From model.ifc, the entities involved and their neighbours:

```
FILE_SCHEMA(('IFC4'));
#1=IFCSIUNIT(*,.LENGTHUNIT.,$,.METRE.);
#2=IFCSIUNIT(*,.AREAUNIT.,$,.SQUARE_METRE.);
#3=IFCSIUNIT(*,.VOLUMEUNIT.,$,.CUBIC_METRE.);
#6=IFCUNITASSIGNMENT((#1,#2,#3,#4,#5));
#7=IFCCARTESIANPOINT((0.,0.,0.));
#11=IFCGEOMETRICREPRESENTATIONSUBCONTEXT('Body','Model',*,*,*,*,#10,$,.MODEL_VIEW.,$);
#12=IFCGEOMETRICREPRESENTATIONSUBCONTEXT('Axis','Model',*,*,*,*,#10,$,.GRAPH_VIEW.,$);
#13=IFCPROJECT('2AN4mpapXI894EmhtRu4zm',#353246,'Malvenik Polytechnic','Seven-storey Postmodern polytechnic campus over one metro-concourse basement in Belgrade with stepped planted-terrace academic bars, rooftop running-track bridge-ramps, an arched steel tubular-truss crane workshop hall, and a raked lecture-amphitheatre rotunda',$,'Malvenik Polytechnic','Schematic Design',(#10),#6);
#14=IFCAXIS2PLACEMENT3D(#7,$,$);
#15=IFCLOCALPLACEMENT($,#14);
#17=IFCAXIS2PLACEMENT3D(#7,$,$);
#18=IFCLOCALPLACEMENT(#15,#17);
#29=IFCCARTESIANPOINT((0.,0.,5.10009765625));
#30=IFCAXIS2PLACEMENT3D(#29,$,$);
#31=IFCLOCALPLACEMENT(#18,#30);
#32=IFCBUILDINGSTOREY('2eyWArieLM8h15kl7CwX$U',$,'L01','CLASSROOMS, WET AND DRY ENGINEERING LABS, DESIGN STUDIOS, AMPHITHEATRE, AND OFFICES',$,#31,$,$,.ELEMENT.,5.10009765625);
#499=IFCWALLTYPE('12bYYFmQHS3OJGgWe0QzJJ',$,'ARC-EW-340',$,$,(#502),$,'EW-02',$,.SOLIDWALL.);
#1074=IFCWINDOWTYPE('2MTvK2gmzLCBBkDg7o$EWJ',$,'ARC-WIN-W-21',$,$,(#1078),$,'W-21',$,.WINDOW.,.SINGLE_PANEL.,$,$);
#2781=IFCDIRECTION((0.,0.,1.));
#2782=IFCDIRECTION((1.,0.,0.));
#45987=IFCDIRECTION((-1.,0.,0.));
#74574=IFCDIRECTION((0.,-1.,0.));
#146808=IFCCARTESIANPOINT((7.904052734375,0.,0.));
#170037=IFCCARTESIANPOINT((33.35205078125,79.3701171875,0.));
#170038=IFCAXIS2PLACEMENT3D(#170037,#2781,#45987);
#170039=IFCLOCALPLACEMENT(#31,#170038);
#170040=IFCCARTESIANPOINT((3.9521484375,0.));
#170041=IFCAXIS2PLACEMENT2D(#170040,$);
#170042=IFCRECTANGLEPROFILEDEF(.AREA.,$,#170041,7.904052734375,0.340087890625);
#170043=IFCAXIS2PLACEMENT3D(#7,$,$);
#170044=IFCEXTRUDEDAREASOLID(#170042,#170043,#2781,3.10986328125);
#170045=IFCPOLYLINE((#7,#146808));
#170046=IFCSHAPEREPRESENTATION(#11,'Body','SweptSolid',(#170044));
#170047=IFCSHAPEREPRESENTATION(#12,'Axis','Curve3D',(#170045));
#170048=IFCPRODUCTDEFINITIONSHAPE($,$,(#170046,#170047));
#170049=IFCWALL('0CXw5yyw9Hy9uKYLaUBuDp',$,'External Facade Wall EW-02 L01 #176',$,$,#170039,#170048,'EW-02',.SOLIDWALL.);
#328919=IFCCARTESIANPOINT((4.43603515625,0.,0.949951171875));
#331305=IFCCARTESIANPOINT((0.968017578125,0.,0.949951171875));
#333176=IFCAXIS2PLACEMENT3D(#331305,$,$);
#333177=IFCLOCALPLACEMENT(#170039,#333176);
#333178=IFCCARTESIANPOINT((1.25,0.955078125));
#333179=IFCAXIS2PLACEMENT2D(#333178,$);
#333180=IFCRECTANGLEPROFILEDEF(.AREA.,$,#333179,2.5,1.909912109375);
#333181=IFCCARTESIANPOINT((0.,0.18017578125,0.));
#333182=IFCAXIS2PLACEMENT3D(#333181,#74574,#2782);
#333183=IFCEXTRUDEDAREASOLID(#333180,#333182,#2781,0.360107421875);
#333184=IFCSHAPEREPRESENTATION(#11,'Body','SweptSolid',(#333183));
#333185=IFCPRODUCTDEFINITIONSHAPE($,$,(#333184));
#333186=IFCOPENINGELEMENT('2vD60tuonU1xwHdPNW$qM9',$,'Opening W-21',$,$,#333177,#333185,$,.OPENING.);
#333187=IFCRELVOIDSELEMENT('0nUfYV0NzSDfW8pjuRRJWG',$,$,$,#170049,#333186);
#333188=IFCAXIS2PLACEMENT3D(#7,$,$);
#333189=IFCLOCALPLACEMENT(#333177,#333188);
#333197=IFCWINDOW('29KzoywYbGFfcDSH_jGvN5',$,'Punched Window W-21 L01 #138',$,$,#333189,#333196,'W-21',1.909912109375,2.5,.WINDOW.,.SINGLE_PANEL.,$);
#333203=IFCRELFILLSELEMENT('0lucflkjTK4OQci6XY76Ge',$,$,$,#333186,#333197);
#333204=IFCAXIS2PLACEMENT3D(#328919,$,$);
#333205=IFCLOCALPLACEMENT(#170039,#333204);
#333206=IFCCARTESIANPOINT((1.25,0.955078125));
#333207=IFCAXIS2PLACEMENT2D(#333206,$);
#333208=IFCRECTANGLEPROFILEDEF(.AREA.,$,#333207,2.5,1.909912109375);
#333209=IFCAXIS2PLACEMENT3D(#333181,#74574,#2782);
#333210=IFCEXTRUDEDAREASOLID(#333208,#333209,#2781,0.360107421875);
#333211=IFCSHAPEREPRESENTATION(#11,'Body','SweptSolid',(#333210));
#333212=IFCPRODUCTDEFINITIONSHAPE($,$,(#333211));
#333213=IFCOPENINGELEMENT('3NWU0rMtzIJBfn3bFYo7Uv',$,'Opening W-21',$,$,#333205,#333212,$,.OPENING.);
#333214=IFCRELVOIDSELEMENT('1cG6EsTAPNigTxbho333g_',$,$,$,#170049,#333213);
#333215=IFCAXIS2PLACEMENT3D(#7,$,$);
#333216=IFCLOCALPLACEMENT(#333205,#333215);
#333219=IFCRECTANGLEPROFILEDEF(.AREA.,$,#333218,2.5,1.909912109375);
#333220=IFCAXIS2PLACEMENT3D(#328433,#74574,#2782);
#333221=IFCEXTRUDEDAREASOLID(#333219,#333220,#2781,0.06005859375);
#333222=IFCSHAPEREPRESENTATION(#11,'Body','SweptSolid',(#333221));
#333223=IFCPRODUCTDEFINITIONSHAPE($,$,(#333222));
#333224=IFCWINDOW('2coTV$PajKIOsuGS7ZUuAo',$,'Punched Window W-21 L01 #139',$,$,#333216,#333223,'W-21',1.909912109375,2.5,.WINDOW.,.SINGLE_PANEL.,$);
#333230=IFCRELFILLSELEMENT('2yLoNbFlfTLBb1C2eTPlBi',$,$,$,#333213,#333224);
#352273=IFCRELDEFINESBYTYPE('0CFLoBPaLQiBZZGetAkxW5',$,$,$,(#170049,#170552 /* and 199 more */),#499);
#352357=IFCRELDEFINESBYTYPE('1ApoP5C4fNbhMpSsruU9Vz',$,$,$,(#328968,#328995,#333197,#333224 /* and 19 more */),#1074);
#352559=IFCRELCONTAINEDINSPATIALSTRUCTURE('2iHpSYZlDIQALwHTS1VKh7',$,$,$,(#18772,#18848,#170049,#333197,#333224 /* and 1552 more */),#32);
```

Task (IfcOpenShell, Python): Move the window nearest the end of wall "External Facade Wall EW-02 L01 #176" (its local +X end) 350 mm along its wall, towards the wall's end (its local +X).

```python
import ifcopenshell
import ifcopenshell.api.geometry
import ifcopenshell.util.placement

model = ifcopenshell.open("model.ifc")

window = model.by_guid("2coTV$PajKIOsuGS7ZUuAo")
opening = window.FillsVoids[0].RelatingOpeningElement
wall = opening.VoidsElements[0].RelatingBuildingElement

wall_matrix = ifcopenshell.util.placement.get_local_placement(wall.ObjectPlacement)
shift = wall_matrix[:3, 0] * 0.35
before = ifcopenshell.util.placement.get_local_placement(window.ObjectPlacement)[:3, 3].copy()

# The window is placed relative to its opening, so it follows when the opening moves.
matrix = ifcopenshell.util.placement.get_local_placement(opening.ObjectPlacement)
matrix[:3, 3] += shift
ifcopenshell.api.geometry.edit_object_placement(
    model, product=opening, matrix=matrix, is_si=False, should_transform_children=True
)

after = ifcopenshell.util.placement.get_local_placement(window.ObjectPlacement)[:3, 3]
print("window moved by", (after - before).round(3) + 0.0)

model.write("model_edited.ifc")
```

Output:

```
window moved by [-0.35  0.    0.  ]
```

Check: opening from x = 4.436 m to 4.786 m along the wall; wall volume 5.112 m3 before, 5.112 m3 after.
